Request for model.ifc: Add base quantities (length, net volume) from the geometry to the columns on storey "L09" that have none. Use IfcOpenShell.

First a look at what the model holds.

```python
import ifcopenshell
import ifcopenshell.util.element
import ifcopenshell.util.unit

model = ifcopenshell.open("model.ifc")
print(model.schema)
for unit_type in ("LENGTHUNIT", "AREAUNIT", "VOLUMEUNIT"):
    print(unit_type, ifcopenshell.util.unit.calculate_unit_scale(model, unit_type))
storey = next(s for s in model.by_type("IfcBuildingStorey") if s.Name == "L09")
columns = [e for e in ifcopenshell.util.element.get_decomposition(storey) if e.is_a("IfcColumn")]
for e in sorted(columns, key=lambda e: e.id()):
    print(e.id(), e.is_a(), e.Name, list(ifcopenshell.util.element.get_psets(e, qtos_only=True)), sep=" | ")
```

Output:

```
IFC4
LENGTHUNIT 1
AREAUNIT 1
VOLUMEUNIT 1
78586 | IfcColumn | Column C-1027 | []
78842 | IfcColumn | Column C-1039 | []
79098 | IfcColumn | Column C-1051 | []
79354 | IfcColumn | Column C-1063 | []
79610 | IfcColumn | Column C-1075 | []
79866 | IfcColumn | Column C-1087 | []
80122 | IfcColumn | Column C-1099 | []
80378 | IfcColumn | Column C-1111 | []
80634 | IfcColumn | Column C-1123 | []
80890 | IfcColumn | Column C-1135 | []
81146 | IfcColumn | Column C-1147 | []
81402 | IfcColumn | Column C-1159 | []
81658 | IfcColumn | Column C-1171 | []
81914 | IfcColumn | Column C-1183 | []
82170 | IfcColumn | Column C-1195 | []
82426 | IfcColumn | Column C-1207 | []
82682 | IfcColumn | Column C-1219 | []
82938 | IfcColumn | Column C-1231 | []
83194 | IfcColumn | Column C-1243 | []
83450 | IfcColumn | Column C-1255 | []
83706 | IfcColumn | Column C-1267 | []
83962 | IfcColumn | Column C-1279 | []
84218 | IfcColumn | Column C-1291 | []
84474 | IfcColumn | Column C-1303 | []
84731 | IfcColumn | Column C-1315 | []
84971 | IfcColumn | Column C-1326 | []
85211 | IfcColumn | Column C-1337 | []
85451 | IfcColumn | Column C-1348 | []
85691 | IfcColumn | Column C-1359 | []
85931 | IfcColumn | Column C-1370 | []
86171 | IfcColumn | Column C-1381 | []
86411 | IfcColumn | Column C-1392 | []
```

```python
import ifcopenshell
import ifcopenshell.api.pset
import ifcopenshell.geom
import ifcopenshell.util.element
import ifcopenshell.util.shape
import ifcopenshell.util.unit

model = ifcopenshell.open("model.ifc")
unit_scale = ifcopenshell.util.unit.calculate_unit_scale(model)
volume_scale = ifcopenshell.util.unit.calculate_unit_scale(model, "VOLUMEUNIT")
settings = ifcopenshell.geom.settings()

storey = next(s for s in model.by_type("IfcBuildingStorey") if s.Name == "L09")
columns = [e for e in ifcopenshell.util.element.get_decomposition(storey) if e.is_a("IfcColumn")]

for e in sorted(columns, key=lambda e: e.id()):
    if ifcopenshell.util.element.get_psets(e, qtos_only=True, should_inherit=False):
        continue
    # Geometry comes back in metres, in the element's own axes.
    shape = ifcopenshell.geom.create_shape(settings, e)
    values = {
        "Length": ifcopenshell.util.shape.get_z(shape.geometry) / unit_scale,
        "NetVolume": ifcopenshell.util.shape.get_volume(shape.geometry) / volume_scale,
    }
    qto = ifcopenshell.api.pset.add_qto(model, product=e, name="Qto_ColumnBaseQuantities")
    ifcopenshell.api.pset.edit_qto(model, qto=qto, properties=values)
    print(e.id(), {k: round(v, 3) for k, v in values.items()})

model.write("model_edited.ifc")
```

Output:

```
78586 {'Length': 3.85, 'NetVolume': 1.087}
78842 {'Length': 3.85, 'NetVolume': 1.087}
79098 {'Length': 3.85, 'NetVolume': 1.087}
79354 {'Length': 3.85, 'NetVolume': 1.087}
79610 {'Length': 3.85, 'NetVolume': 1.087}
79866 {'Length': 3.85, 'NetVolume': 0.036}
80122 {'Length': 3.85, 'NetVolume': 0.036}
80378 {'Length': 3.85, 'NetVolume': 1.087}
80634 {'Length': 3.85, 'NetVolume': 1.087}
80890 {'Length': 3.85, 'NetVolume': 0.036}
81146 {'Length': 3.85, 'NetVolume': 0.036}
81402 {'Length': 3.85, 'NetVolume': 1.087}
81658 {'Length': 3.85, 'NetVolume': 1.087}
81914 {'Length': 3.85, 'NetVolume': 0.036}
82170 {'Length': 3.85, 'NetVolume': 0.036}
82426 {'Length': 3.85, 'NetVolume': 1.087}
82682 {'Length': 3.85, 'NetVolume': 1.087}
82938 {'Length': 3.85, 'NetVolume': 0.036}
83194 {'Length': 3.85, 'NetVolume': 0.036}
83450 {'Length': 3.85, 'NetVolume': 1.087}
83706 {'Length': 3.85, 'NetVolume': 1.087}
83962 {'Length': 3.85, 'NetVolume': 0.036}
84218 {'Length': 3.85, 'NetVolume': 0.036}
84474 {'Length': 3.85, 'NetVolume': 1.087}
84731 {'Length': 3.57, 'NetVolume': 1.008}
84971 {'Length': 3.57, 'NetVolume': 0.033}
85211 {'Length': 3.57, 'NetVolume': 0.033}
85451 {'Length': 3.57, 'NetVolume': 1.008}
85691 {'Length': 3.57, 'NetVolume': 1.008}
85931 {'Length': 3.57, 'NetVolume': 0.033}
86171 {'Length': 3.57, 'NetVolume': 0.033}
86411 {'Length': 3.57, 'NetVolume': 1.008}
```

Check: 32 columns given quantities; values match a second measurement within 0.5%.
